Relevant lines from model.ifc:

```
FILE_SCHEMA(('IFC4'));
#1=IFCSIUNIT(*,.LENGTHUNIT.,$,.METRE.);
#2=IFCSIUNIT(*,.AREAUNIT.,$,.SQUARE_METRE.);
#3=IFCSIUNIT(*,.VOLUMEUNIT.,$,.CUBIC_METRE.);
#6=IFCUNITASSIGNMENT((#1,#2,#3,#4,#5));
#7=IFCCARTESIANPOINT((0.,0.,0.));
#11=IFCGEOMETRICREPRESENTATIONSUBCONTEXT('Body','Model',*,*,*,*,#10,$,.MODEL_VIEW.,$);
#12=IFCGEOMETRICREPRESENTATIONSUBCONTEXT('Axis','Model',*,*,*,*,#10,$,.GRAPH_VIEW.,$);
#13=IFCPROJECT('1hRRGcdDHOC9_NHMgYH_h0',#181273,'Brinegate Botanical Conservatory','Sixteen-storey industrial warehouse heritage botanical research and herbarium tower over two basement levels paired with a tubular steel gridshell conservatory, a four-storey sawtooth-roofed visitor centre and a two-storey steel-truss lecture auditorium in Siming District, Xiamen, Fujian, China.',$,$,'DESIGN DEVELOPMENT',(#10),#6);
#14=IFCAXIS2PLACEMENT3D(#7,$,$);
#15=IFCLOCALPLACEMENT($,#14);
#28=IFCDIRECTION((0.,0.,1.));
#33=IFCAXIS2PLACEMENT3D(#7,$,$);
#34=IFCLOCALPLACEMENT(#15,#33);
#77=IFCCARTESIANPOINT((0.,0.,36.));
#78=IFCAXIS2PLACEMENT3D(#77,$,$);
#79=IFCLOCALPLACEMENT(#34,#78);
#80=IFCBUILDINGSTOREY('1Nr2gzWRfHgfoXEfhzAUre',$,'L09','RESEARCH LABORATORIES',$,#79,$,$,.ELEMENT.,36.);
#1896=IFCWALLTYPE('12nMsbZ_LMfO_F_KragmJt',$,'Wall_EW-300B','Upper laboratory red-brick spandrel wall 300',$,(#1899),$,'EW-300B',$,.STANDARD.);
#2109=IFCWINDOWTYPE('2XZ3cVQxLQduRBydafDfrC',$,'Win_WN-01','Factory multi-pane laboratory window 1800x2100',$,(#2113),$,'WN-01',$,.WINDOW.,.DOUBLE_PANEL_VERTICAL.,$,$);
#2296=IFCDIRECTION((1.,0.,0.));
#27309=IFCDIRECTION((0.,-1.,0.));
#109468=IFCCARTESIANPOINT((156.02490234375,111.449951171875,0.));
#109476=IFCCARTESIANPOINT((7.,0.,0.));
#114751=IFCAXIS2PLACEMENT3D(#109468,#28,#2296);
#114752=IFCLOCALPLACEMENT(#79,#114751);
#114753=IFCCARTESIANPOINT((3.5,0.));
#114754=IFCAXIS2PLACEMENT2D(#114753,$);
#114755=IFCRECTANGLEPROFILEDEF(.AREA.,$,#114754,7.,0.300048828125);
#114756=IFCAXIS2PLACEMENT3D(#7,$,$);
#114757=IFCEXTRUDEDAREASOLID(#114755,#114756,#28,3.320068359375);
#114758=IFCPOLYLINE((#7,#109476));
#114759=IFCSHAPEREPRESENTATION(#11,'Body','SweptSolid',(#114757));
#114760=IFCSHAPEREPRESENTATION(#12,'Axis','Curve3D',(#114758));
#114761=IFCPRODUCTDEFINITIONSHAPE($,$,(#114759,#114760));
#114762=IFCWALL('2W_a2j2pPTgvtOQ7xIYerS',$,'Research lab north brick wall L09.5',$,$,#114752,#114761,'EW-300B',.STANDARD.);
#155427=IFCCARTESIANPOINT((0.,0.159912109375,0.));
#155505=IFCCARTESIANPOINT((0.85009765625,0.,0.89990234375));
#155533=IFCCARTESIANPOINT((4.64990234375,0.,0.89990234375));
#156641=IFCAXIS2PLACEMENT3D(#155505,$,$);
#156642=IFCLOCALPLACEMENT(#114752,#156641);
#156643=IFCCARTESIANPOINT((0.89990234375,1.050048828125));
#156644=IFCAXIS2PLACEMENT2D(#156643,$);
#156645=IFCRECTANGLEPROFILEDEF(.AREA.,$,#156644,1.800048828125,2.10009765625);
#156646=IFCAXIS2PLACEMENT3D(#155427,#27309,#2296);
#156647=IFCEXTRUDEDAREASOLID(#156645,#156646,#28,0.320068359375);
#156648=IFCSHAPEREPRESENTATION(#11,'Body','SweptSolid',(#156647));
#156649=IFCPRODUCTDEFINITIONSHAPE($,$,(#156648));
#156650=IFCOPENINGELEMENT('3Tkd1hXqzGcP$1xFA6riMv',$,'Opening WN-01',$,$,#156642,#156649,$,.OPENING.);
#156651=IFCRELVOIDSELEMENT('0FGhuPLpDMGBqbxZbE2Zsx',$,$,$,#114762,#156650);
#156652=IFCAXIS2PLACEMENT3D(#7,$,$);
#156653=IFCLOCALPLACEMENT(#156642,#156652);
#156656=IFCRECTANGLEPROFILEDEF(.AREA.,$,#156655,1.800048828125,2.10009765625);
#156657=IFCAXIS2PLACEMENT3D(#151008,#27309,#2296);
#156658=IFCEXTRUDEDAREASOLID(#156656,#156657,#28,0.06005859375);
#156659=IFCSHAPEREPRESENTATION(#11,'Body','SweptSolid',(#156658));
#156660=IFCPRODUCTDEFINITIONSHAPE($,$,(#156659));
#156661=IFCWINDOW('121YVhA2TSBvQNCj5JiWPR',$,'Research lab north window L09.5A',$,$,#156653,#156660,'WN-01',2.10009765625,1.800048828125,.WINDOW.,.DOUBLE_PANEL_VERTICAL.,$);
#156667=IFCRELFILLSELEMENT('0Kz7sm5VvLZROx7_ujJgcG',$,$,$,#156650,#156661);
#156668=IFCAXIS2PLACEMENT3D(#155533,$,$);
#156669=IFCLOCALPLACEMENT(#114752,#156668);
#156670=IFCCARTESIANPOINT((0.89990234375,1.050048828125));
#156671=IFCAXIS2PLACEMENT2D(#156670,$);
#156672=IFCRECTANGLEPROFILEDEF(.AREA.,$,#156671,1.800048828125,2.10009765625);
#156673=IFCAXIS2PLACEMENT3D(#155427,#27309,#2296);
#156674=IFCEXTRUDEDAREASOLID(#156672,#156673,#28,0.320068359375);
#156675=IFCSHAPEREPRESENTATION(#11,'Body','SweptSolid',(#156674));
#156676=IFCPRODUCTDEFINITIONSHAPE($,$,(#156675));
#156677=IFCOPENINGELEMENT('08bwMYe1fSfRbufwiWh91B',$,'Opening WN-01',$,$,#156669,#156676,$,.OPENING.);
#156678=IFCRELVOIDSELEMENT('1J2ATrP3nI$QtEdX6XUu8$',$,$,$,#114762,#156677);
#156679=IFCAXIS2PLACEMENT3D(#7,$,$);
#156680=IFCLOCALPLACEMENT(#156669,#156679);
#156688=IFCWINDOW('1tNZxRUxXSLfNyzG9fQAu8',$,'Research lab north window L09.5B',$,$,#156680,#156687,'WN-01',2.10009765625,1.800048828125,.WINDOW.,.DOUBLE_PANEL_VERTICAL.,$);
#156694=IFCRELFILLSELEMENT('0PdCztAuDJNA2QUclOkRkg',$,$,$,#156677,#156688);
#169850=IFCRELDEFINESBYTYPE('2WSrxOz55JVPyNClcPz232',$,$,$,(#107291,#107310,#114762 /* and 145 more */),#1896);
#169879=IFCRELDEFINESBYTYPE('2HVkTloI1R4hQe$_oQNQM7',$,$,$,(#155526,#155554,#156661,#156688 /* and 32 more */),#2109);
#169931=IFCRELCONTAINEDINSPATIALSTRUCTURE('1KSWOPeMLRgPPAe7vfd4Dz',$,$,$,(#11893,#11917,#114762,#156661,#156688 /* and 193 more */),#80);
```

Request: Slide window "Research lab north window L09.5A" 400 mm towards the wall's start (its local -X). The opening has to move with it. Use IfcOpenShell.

```python
import ifcopenshell
import ifcopenshell.api.geometry
import ifcopenshell.util.placement

model = ifcopenshell.open("model.ifc")

window = model.by_guid("121YVhA2TSBvQNCj5JiWPR")
opening = window.FillsVoids[0].RelatingOpeningElement
wall = opening.VoidsElements[0].RelatingBuildingElement

wall_matrix = ifcopenshell.util.placement.get_local_placement(wall.ObjectPlacement)
shift = wall_matrix[:3, 0] * -0.4
before = ifcopenshell.util.placement.get_local_placement(window.ObjectPlacement)[:3, 3].copy()

# The window is placed relative to its opening, so it follows when the opening moves.
matrix = ifcopenshell.util.placement.get_local_placement(opening.ObjectPlacement)
matrix[:3, 3] += shift
ifcopenshell.api.geometry.edit_object_placement(
    model, product=opening, matrix=matrix, is_si=False, should_transform_children=True
)

after = ifcopenshell.util.placement.get_local_placement(window.ObjectPlacement)[:3, 3]
print("window moved by", (after - before).round(3) + 0.0)

model.write("model_v2.ifc")
```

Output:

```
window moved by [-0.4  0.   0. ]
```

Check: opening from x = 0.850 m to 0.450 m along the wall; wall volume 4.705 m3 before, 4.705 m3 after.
